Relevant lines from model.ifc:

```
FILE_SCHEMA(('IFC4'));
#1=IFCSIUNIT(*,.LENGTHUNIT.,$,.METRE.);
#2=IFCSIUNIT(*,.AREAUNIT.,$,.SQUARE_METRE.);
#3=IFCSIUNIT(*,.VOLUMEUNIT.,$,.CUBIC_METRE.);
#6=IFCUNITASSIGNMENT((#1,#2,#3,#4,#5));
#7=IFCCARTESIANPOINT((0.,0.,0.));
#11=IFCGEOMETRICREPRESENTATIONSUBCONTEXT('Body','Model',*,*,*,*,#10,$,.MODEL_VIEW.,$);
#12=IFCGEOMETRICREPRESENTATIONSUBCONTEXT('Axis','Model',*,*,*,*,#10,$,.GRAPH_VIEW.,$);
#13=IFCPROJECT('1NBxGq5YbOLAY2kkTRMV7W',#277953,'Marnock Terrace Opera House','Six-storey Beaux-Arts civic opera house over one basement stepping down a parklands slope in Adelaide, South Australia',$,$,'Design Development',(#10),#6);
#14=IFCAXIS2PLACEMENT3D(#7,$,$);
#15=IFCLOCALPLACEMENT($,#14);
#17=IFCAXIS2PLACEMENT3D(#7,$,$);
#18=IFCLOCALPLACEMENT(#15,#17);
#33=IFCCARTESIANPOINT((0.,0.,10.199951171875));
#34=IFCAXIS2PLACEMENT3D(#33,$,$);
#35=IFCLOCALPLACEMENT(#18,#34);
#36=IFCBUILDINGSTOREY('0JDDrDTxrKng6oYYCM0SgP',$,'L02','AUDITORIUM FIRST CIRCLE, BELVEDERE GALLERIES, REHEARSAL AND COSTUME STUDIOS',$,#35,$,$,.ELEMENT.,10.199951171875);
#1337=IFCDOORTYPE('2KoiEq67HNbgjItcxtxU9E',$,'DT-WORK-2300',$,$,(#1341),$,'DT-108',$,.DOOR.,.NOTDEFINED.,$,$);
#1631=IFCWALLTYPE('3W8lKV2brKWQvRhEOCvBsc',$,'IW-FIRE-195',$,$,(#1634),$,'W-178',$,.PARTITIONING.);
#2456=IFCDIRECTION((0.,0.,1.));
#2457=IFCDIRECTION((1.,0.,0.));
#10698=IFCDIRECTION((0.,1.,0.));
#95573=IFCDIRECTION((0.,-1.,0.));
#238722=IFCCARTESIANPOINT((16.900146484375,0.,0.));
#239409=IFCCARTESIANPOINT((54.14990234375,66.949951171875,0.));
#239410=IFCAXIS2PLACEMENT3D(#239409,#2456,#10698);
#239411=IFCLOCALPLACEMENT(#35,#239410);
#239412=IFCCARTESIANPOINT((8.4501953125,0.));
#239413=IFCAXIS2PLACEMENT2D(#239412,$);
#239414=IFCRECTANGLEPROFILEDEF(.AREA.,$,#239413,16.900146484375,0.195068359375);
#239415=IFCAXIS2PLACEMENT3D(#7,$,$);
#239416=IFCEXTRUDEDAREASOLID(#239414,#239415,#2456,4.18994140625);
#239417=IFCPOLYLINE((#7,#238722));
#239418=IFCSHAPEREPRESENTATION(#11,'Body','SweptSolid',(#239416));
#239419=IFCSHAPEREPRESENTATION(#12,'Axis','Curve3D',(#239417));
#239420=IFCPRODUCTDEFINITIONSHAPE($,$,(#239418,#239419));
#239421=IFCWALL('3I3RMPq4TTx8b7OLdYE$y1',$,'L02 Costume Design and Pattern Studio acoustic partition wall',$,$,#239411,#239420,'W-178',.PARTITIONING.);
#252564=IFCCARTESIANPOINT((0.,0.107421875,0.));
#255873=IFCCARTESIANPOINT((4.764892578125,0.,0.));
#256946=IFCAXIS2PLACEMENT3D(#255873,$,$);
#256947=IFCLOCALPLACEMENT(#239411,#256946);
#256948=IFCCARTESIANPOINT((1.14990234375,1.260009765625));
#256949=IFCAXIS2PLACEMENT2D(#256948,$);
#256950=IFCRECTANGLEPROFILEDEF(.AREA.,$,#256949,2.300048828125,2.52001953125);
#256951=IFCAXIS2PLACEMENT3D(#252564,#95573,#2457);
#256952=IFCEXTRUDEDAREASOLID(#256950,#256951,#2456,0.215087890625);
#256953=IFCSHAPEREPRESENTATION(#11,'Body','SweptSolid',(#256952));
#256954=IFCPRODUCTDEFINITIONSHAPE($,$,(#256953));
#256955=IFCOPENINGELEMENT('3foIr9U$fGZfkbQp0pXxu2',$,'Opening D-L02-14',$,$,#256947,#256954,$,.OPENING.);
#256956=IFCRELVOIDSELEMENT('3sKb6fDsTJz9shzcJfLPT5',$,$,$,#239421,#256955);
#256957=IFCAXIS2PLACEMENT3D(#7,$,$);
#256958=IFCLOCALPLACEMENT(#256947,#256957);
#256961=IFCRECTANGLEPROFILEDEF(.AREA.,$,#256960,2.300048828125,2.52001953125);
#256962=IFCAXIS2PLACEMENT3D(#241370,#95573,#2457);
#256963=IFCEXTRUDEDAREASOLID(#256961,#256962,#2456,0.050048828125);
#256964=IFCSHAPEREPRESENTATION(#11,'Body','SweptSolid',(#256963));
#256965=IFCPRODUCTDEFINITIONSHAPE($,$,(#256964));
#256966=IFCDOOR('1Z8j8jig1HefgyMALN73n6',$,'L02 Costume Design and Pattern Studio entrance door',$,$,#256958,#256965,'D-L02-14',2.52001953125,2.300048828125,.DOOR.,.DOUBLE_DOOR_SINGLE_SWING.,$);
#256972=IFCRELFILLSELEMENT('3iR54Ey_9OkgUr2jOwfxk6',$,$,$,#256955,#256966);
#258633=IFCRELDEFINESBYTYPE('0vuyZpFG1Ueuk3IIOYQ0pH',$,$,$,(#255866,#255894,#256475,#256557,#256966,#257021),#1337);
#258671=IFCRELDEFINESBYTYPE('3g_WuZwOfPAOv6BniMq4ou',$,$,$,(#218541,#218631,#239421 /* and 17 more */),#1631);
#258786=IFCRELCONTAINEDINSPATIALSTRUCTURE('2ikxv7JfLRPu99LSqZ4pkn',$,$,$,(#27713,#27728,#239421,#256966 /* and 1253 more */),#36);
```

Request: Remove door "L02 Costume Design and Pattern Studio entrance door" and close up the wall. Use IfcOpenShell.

```python
import ifcopenshell
import ifcopenshell.api.feature
import ifcopenshell.api.root
import ifcopenshell.geom
import ifcopenshell.util.shape

model = ifcopenshell.open("model.ifc")
settings = ifcopenshell.geom.settings()


def volume(element):
    """Net volume in cubic metres, openings subtracted."""
    shape = ifcopenshell.geom.create_shape(settings, element)
    return ifcopenshell.util.shape.get_volume(shape.geometry)


door = model.by_guid("1Z8j8jig1HefgyMALN73n6")
opening = door.FillsVoids[0].RelatingOpeningElement
wall = opening.VoidsElements[0].RelatingBuildingElement
before = volume(wall)

ifcopenshell.api.root.remove_product(model, product=door)
ifcopenshell.api.feature.remove_feature(model, feature=opening)

after = volume(wall)

print(f"wall volume {before:.3f} -> {after:.3f} m3")

model.write("model_rev.ifc")
```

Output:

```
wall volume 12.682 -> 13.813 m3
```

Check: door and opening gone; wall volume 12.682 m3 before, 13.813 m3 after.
